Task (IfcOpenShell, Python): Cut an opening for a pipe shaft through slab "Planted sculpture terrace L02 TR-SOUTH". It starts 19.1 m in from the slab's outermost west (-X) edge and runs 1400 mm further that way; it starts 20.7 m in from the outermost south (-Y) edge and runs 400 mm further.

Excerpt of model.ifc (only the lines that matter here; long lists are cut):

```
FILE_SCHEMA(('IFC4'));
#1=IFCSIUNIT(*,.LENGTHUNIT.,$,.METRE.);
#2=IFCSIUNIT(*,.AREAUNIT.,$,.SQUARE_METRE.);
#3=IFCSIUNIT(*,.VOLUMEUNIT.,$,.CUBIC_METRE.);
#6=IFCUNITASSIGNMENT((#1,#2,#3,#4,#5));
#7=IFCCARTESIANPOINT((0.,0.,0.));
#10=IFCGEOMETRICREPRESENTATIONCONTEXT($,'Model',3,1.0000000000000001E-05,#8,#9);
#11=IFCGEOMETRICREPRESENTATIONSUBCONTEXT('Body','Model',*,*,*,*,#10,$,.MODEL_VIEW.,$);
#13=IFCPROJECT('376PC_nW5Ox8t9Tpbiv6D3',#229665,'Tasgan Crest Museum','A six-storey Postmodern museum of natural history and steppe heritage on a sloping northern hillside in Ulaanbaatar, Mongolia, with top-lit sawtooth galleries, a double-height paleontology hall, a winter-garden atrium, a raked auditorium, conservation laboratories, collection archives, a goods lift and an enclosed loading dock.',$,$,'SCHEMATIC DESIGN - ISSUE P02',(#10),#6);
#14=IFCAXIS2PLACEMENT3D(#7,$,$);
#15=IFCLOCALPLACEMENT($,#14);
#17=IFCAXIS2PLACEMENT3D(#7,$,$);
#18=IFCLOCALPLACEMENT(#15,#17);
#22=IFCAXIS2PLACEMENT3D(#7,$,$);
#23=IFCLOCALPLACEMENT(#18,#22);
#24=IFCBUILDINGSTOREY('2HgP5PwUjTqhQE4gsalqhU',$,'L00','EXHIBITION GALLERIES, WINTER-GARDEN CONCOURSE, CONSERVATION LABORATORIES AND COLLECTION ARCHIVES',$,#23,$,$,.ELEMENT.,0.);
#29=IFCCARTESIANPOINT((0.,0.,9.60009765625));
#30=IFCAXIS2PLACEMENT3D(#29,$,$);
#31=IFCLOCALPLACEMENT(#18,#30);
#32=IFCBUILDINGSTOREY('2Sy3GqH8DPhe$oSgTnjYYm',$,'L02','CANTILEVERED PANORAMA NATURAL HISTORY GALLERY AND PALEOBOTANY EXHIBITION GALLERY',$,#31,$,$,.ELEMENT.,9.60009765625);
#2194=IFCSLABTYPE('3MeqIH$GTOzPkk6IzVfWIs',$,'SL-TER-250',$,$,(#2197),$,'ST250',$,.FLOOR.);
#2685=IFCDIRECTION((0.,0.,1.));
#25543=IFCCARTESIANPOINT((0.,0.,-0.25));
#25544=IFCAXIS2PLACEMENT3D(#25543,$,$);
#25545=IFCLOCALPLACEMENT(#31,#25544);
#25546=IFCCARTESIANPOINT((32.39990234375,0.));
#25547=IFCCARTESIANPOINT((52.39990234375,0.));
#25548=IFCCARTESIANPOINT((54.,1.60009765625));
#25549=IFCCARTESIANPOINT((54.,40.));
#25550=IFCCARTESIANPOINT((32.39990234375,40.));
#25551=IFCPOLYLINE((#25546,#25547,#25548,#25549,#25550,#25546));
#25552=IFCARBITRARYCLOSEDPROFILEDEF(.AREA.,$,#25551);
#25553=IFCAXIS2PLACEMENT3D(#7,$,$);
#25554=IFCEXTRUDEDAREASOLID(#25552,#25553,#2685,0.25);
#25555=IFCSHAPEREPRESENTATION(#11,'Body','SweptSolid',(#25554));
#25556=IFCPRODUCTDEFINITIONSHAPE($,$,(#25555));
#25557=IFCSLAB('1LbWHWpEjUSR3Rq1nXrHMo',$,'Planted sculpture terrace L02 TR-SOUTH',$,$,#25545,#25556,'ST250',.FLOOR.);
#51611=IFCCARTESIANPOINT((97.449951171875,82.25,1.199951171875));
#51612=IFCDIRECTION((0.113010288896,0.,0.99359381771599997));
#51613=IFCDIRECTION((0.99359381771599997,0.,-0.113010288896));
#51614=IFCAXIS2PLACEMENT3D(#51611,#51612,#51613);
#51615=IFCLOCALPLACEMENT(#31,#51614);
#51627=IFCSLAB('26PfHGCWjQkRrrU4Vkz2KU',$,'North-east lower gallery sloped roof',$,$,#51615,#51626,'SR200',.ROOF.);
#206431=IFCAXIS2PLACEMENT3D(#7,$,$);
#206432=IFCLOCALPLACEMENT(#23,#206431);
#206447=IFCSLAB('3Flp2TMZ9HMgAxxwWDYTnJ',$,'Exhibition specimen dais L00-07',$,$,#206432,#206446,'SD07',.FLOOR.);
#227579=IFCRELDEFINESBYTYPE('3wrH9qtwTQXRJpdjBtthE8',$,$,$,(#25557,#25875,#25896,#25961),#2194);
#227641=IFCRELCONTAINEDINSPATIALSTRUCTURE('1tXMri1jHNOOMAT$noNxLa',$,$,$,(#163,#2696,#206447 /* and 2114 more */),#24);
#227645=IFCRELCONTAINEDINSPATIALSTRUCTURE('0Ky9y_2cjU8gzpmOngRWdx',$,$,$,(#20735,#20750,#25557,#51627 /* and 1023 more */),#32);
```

```python
import numpy as np
import ifcopenshell
import ifcopenshell.api.feature
import ifcopenshell.api.geometry
import ifcopenshell.api.root
import ifcopenshell.geom
import ifcopenshell.util.placement
import ifcopenshell.util.representation
import ifcopenshell.util.shape
import ifcopenshell.util.unit

model = ifcopenshell.open("model.ifc")
unit_scale = ifcopenshell.util.unit.calculate_unit_scale(model)
settings = ifcopenshell.geom.settings()


def volume(element):
    """Net volume in cubic metres, openings subtracted."""
    shape = ifcopenshell.geom.create_shape(settings, element)
    return ifcopenshell.util.shape.get_volume(shape.geometry)


slab = model.by_guid("1LbWHWpEjUSR3Rq1nXrHMo")
before = volume(slab)

# Extent in the slab's own axes, in metres. The edges named are its -X and -Y sides.
slab_shape = ifcopenshell.geom.create_shape(settings, slab)
vertices = ifcopenshell.util.shape.get_vertices(slab_shape.geometry)
x_min, y_min, bottom = vertices.min(axis=0)
top = vertices[:, 2].max()

opening = ifcopenshell.api.root.create_entity(model, ifc_class="IfcOpeningElement", name="Pipe shaft opening", predefined_type="OPENING")
context = ifcopenshell.util.representation.get_context(model, "Model", "Body", "MODEL_VIEW")
width, depth = 1.4, 0.4
outline = [(0.0, 0.0), (width, 0.0), (width, depth), (0.0, depth), (0.0, 0.0)]
# Overshoot both faces by 50 mm so the cut is clean.
shape = ifcopenshell.api.geometry.add_slab_representation(
    model, context=context, depth=top - bottom + 0.1, polyline=outline
)
ifcopenshell.api.geometry.assign_representation(model, product=opening, representation=shape)

matrix = ifcopenshell.util.placement.get_local_placement(slab.ObjectPlacement)
matrix[:, 3] = matrix @ np.append(np.array([x_min + 19.1, y_min + 20.7, bottom - 0.05]) / unit_scale, 1.0)
ifcopenshell.api.geometry.edit_object_placement(model, product=opening, matrix=matrix, is_si=False)
ifcopenshell.api.feature.add_feature(model, feature=opening, element=slab)

after = volume(slab)

print(f"slab volume {before:.3f} -> {after:.3f} m3")

model.write("model-out.ifc")
```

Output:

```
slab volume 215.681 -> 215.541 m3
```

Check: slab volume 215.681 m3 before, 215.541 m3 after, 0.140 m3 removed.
